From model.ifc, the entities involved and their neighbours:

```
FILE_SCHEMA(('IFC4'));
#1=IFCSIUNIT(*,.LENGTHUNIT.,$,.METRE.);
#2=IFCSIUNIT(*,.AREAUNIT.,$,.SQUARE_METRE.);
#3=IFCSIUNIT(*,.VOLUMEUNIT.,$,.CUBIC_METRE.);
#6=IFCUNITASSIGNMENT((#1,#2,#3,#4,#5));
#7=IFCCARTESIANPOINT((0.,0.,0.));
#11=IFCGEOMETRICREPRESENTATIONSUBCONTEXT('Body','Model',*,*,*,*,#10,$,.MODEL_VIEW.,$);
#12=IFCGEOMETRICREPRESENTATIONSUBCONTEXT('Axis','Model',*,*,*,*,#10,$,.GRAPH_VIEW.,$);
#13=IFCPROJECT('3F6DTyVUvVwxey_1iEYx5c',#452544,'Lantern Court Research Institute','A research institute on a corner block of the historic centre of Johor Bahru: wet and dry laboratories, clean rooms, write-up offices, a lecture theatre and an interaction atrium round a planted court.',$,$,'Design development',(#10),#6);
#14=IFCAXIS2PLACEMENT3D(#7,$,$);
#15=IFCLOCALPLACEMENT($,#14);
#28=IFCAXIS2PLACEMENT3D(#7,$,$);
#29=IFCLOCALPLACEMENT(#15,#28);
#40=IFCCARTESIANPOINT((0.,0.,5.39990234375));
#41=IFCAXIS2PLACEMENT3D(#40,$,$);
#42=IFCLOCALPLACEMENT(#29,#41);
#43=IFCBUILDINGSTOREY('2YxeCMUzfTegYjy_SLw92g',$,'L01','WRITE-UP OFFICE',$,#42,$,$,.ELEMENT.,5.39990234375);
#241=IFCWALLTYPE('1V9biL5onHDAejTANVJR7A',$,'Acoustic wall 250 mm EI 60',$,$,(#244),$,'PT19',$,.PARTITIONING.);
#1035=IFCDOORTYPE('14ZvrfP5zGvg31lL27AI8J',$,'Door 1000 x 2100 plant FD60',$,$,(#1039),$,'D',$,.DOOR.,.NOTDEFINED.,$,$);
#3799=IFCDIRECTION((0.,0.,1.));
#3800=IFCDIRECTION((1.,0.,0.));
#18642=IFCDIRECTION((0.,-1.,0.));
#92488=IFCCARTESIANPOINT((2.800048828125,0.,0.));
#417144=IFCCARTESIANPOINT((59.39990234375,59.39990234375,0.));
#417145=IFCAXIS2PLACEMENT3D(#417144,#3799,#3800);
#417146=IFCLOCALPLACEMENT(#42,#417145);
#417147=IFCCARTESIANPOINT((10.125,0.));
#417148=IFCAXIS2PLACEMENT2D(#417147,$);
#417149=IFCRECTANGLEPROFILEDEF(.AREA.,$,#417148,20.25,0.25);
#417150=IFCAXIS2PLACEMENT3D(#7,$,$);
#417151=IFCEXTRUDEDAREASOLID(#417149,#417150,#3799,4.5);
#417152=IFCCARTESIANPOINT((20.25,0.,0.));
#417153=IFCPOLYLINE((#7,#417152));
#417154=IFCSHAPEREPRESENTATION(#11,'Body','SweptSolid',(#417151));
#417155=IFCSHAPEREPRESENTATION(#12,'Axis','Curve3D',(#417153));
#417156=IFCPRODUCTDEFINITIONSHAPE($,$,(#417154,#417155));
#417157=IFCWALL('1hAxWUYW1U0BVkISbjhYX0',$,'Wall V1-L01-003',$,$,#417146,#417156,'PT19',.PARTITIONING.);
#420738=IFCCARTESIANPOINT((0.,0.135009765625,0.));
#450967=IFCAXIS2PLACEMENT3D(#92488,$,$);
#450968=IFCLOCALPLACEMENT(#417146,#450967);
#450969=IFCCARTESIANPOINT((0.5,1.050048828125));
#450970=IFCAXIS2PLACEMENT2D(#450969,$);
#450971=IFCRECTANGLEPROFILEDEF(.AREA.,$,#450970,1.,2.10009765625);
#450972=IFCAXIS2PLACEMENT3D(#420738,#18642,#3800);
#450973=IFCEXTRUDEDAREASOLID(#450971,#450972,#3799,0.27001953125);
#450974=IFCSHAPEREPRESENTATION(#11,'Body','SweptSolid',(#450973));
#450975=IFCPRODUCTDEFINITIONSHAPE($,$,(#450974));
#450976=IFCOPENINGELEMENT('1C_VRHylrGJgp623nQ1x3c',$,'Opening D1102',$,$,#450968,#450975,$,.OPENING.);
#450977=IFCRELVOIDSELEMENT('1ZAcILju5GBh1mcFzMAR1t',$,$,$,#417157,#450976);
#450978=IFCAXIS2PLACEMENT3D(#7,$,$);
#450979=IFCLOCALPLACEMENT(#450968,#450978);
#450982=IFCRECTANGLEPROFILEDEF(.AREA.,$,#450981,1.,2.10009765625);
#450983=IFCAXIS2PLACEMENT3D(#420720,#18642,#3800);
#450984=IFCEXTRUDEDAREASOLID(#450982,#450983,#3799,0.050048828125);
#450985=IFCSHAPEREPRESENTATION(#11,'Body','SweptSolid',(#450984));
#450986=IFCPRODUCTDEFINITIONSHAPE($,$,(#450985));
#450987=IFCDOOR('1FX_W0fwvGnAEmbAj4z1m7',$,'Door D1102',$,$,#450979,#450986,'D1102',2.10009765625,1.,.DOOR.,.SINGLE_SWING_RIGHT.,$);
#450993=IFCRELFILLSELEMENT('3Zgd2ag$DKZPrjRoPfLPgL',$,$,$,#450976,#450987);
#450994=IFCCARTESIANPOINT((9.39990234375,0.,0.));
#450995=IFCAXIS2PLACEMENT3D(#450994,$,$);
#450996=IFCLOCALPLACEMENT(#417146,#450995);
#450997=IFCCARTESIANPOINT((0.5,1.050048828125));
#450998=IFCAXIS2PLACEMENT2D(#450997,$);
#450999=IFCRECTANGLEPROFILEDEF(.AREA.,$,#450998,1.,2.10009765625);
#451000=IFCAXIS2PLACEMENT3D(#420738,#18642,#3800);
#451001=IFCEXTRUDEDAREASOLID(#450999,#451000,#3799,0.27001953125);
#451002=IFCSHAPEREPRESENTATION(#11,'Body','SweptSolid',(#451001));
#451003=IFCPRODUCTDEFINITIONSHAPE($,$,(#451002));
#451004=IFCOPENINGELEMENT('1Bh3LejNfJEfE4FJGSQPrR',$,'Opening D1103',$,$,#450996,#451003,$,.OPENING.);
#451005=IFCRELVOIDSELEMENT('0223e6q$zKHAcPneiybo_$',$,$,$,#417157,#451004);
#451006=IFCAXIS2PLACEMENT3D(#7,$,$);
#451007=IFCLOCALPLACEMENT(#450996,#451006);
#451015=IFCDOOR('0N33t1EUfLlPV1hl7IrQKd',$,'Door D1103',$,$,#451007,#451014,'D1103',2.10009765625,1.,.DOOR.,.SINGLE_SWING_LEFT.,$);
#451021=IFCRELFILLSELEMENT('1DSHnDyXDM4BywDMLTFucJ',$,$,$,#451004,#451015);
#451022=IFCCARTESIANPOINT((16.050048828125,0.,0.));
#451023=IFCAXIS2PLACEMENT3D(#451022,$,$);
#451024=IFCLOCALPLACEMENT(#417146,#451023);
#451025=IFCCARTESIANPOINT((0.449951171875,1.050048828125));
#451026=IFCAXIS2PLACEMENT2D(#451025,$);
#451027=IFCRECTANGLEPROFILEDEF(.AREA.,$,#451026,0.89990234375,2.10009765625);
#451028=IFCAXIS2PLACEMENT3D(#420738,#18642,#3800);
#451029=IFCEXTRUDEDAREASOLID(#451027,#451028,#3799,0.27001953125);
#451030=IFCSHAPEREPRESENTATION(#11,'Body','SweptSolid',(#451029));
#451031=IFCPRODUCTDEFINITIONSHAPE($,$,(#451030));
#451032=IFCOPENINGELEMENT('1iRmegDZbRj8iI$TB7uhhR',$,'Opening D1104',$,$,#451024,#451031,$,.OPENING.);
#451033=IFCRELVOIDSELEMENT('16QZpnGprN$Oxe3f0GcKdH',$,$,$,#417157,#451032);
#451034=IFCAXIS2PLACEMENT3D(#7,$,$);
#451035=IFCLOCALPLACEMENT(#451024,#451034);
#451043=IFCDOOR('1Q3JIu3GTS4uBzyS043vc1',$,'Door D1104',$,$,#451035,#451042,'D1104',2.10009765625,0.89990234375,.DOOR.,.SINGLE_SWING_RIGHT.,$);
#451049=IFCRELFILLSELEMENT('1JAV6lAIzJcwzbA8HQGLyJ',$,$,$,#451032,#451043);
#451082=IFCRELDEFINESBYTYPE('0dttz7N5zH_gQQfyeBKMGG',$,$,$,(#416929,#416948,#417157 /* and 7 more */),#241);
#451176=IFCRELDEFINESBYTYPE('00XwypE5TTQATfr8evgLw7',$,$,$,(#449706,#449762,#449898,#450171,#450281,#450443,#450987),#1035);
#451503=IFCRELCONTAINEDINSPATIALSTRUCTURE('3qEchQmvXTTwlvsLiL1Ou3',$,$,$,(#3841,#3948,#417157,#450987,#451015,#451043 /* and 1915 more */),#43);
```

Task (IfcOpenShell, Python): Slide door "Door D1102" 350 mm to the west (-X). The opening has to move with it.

```python
import ifcopenshell
import ifcopenshell.api.geometry
import ifcopenshell.util.placement
import ifcopenshell.util.unit

model = ifcopenshell.open("model.ifc")
unit_scale = ifcopenshell.util.unit.calculate_unit_scale(model)

door = model.by_guid("1FX_W0fwvGnAEmbAj4z1m7")
opening = door.FillsVoids[0].RelatingOpeningElement
wall = opening.VoidsElements[0].RelatingBuildingElement

wall_matrix = ifcopenshell.util.placement.get_local_placement(wall.ObjectPlacement)
shift = wall_matrix[:3, 0] * -0.35 / unit_scale
before = ifcopenshell.util.placement.get_local_placement(door.ObjectPlacement)[:3, 3].copy()

# The door is placed relative to its opening, so it follows when the opening moves.
matrix = ifcopenshell.util.placement.get_local_placement(opening.ObjectPlacement)
matrix[:3, 3] += shift
ifcopenshell.api.geometry.edit_object_placement(
    model, product=opening, matrix=matrix, is_si=False, should_transform_children=True
)

after = ifcopenshell.util.placement.get_local_placement(door.ObjectPlacement)[:3, 3]
print("door moved by", (after - before).round(3) + 0.0)

model.write("model_updated.ifc")
```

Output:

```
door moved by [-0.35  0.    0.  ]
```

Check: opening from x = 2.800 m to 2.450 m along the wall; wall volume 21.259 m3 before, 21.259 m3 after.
